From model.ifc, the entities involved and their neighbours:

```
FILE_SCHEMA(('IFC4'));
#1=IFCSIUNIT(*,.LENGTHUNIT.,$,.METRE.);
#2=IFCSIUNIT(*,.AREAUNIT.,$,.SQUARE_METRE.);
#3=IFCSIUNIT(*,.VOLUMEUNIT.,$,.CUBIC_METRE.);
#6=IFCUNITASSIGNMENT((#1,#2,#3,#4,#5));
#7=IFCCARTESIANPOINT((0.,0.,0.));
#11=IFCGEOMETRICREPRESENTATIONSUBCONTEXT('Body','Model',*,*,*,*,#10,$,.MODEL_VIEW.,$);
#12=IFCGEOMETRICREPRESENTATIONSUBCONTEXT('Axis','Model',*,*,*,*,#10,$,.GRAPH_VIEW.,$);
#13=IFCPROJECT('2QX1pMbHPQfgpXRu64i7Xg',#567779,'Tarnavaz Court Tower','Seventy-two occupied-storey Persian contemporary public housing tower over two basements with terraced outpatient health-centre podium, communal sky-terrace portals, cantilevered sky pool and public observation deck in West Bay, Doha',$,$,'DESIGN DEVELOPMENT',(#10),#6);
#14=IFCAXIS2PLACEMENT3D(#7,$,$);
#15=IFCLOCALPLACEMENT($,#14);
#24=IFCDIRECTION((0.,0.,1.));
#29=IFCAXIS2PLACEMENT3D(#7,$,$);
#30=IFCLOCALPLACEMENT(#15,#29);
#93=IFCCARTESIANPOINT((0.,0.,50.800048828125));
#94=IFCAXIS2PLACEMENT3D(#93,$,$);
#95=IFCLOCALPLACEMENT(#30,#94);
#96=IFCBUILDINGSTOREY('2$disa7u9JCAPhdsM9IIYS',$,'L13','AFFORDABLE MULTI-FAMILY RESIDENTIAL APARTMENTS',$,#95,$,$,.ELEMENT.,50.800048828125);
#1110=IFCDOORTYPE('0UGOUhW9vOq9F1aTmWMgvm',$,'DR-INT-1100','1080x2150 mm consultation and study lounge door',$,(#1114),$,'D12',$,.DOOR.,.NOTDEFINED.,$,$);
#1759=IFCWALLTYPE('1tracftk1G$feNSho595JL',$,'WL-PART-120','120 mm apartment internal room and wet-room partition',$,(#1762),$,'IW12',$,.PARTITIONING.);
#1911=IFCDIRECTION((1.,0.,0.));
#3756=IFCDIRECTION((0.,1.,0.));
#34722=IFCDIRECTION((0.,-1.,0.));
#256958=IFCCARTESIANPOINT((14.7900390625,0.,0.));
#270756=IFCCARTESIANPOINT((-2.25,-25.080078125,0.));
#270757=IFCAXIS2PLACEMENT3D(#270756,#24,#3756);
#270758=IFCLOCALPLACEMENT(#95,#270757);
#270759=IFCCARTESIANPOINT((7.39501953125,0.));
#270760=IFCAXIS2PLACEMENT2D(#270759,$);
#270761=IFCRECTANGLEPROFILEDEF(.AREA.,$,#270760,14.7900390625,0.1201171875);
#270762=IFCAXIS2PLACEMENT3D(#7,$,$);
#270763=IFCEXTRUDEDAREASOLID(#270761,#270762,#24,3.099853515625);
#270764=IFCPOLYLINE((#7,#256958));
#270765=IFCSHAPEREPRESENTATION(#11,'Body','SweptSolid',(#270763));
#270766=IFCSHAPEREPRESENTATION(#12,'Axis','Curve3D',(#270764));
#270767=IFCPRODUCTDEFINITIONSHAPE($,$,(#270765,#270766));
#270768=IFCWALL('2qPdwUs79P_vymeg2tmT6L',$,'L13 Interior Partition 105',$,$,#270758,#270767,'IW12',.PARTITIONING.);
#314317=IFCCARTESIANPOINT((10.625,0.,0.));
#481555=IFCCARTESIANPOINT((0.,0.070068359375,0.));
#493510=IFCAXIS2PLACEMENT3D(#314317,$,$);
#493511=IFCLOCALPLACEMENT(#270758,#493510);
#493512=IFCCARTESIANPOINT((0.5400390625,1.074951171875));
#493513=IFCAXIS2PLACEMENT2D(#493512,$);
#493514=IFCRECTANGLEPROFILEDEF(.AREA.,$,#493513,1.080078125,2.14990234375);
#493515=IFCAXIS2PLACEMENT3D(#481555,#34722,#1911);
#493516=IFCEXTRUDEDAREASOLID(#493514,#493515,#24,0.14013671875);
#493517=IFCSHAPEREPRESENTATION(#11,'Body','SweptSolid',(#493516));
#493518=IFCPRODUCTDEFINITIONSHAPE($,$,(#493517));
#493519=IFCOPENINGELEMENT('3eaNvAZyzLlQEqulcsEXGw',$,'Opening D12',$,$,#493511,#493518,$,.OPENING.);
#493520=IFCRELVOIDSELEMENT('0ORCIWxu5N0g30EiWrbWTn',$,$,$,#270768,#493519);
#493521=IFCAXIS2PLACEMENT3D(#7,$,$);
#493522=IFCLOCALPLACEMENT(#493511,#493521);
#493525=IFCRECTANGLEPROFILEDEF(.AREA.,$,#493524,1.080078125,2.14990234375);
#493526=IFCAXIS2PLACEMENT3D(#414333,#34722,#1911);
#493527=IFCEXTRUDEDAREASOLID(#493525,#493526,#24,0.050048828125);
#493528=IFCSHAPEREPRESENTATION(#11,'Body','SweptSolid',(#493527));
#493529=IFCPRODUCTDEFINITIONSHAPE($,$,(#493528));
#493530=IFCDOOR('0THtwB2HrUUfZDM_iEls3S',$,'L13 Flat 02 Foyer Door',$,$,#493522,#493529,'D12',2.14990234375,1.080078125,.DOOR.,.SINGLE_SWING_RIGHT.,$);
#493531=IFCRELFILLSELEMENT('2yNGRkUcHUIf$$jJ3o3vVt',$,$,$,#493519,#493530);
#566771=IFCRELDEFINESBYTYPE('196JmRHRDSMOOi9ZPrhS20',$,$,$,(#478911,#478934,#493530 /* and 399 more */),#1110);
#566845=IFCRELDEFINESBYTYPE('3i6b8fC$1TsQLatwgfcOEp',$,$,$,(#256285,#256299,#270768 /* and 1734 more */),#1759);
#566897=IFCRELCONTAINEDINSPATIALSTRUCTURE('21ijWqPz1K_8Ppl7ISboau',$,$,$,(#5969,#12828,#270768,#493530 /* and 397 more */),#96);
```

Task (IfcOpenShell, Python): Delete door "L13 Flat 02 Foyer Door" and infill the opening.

```python
import ifcopenshell
import ifcopenshell.api.feature
import ifcopenshell.api.root
import ifcopenshell.geom
import ifcopenshell.util.shape

model = ifcopenshell.open("model.ifc")
settings = ifcopenshell.geom.settings()


def volume(element):
    """Net volume in cubic metres, openings subtracted."""
    shape = ifcopenshell.geom.create_shape(settings, element)
    return ifcopenshell.util.shape.get_volume(shape.geometry)


door = model.by_id(493530)
opening = door.FillsVoids[0].RelatingOpeningElement
wall = opening.VoidsElements[0].RelatingBuildingElement
before = volume(wall)

ifcopenshell.api.root.remove_product(model, product=door)
ifcopenshell.api.feature.remove_feature(model, feature=opening)

after = volume(wall)

print(f"wall volume {before:.3f} -> {after:.3f} m3")

model.write("model_updated.ifc")
```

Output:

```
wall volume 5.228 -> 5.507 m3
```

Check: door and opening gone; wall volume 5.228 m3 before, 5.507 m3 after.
